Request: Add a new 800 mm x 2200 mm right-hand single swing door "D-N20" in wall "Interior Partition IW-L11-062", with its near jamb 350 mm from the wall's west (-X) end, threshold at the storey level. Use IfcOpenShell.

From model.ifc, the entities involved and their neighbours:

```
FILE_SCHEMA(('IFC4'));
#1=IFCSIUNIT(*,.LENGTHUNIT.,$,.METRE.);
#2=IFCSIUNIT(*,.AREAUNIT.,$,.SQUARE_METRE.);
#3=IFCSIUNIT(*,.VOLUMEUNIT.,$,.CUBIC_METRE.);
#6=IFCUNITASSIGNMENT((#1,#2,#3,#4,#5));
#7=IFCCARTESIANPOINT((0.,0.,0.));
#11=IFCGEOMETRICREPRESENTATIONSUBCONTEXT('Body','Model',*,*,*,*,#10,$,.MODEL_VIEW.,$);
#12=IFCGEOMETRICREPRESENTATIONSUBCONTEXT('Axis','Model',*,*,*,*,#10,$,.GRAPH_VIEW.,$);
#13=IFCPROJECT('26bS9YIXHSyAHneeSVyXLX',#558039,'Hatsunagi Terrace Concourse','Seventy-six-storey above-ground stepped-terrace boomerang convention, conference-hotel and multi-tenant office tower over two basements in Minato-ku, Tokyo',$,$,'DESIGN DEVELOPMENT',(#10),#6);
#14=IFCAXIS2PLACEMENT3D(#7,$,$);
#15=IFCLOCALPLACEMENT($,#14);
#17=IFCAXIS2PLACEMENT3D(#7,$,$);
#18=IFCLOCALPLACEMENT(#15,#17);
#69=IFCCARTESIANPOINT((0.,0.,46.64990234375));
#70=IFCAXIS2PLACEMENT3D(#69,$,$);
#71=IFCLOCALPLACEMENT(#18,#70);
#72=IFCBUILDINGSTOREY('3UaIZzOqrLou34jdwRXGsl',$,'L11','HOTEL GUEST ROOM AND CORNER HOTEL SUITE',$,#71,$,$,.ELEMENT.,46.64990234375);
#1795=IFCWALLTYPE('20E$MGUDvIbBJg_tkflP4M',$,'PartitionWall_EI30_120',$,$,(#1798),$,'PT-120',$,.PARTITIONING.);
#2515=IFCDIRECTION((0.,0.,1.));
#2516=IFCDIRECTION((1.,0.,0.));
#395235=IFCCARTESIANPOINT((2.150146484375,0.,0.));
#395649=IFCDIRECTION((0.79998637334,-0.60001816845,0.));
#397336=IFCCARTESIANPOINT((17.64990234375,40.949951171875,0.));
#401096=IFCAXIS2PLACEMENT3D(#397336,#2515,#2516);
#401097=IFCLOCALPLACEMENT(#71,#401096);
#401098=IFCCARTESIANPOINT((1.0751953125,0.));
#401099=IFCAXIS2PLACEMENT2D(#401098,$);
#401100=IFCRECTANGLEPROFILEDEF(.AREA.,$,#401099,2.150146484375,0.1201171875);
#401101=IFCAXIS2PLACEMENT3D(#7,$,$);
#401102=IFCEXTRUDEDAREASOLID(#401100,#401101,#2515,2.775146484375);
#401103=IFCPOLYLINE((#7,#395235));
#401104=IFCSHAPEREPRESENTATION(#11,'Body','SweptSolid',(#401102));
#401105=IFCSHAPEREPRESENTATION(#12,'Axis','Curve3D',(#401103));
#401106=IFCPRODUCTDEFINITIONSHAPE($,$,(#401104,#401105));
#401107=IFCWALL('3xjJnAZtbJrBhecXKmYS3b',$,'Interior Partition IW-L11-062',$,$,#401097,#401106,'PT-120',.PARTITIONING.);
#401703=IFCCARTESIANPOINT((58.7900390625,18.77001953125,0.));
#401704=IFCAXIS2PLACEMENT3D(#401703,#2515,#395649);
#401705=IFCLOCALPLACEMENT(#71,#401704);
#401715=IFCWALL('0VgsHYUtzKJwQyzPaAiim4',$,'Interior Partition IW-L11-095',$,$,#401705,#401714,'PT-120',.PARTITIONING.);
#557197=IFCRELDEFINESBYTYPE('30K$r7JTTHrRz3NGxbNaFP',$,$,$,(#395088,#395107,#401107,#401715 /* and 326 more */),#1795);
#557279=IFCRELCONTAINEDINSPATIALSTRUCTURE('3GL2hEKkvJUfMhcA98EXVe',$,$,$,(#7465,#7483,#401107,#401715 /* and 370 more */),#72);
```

```python
import numpy as np
import ifcopenshell
import ifcopenshell.api.feature
import ifcopenshell.api.geometry
import ifcopenshell.api.root
import ifcopenshell.api.spatial
import ifcopenshell.geom
import ifcopenshell.util.element
import ifcopenshell.util.placement
import ifcopenshell.util.representation
import ifcopenshell.util.shape
import ifcopenshell.util.unit

model = ifcopenshell.open("model.ifc")
unit_scale = ifcopenshell.util.unit.calculate_unit_scale(model)
settings = ifcopenshell.geom.settings()


def volume(element):
    """Net volume in cubic metres, openings subtracted."""
    shape = ifcopenshell.geom.create_shape(settings, element)
    return ifcopenshell.util.shape.get_volume(shape.geometry)


wall = model.by_guid("3xjJnAZtbJrBhecXKmYS3b")
storey = ifcopenshell.util.element.get_container(wall, ifc_class="IfcBuildingStorey")
context = ifcopenshell.util.representation.get_context(model, "Model", "Body", "MODEL_VIEW")
before = volume(wall)

width, height, from_end, sill = 0.8, 2.2, 0.35, 0.0  # metres

# The wall runs along its own X axis, and the end named is its -X end.
wall_shape = ifcopenshell.geom.create_shape(settings, wall)
x, y, z = ifcopenshell.util.shape.get_vertices(wall_shape.geometry).T
start = x.min() + from_end
face, thickness = float(y.min()), float(y.max() - y.min())
wall_matrix = ifcopenshell.util.placement.get_local_placement(wall.ObjectPlacement)
level = ifcopenshell.util.placement.get_local_placement(storey.ObjectPlacement)[2, 3]


def in_wall(x, y):
    """Placement at x, y metres in the wall's axes, at sill height."""
    matrix = wall_matrix.copy()
    matrix[:, 3] = wall_matrix @ np.array([x / unit_scale, y / unit_scale, 0.0, 1.0])
    matrix[2, 3] = level + sill / unit_scale
    return matrix


# Opening: a box that overshoots both wall faces by 50 mm.
opening = ifcopenshell.api.root.create_entity(model, ifc_class="IfcOpeningElement", predefined_type="OPENING")
box = ifcopenshell.api.geometry.add_wall_representation(
    model, context=context, length=width, height=height, thickness=thickness + 0.1
)
ifcopenshell.api.geometry.assign_representation(model, product=opening, representation=box)
ifcopenshell.api.geometry.edit_object_placement(model, product=opening, matrix=in_wall(start, face - 0.05), is_si=False)
ifcopenshell.api.feature.add_feature(model, feature=opening, element=wall)

door = ifcopenshell.api.root.create_entity(model, ifc_class="IfcDoor", name="D-N20", predefined_type="DOOR")
door.OverallWidth, door.OverallHeight = width / unit_scale, height / unit_scale
door.OperationType = "SINGLE_SWING_RIGHT"
body = ifcopenshell.api.geometry.add_door_representation(
    model,
    context=context,
    overall_width=door.OverallWidth,
    overall_height=door.OverallHeight,
    operation_type="SINGLE_SWING_RIGHT",
    lining_properties={"LiningDepth": thickness / unit_scale, "ThresholdDepth": thickness / unit_scale},
)
ifcopenshell.api.geometry.assign_representation(model, product=door, representation=body)
ifcopenshell.api.spatial.assign_container(model, products=[door], relating_structure=storey)
ifcopenshell.api.feature.add_filling(model, opening=opening, element=door)

# The lining spans the wall, so the door starts at the wall face.
ifcopenshell.api.geometry.edit_object_placement(model, product=door, matrix=in_wall(start, face), is_si=False)

after = volume(wall)

print(f"wall volume {before:.3f} -> {after:.3f} m3")

model.write("model_rev.ifc")
```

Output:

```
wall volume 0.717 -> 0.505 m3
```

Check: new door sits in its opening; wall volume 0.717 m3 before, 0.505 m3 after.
